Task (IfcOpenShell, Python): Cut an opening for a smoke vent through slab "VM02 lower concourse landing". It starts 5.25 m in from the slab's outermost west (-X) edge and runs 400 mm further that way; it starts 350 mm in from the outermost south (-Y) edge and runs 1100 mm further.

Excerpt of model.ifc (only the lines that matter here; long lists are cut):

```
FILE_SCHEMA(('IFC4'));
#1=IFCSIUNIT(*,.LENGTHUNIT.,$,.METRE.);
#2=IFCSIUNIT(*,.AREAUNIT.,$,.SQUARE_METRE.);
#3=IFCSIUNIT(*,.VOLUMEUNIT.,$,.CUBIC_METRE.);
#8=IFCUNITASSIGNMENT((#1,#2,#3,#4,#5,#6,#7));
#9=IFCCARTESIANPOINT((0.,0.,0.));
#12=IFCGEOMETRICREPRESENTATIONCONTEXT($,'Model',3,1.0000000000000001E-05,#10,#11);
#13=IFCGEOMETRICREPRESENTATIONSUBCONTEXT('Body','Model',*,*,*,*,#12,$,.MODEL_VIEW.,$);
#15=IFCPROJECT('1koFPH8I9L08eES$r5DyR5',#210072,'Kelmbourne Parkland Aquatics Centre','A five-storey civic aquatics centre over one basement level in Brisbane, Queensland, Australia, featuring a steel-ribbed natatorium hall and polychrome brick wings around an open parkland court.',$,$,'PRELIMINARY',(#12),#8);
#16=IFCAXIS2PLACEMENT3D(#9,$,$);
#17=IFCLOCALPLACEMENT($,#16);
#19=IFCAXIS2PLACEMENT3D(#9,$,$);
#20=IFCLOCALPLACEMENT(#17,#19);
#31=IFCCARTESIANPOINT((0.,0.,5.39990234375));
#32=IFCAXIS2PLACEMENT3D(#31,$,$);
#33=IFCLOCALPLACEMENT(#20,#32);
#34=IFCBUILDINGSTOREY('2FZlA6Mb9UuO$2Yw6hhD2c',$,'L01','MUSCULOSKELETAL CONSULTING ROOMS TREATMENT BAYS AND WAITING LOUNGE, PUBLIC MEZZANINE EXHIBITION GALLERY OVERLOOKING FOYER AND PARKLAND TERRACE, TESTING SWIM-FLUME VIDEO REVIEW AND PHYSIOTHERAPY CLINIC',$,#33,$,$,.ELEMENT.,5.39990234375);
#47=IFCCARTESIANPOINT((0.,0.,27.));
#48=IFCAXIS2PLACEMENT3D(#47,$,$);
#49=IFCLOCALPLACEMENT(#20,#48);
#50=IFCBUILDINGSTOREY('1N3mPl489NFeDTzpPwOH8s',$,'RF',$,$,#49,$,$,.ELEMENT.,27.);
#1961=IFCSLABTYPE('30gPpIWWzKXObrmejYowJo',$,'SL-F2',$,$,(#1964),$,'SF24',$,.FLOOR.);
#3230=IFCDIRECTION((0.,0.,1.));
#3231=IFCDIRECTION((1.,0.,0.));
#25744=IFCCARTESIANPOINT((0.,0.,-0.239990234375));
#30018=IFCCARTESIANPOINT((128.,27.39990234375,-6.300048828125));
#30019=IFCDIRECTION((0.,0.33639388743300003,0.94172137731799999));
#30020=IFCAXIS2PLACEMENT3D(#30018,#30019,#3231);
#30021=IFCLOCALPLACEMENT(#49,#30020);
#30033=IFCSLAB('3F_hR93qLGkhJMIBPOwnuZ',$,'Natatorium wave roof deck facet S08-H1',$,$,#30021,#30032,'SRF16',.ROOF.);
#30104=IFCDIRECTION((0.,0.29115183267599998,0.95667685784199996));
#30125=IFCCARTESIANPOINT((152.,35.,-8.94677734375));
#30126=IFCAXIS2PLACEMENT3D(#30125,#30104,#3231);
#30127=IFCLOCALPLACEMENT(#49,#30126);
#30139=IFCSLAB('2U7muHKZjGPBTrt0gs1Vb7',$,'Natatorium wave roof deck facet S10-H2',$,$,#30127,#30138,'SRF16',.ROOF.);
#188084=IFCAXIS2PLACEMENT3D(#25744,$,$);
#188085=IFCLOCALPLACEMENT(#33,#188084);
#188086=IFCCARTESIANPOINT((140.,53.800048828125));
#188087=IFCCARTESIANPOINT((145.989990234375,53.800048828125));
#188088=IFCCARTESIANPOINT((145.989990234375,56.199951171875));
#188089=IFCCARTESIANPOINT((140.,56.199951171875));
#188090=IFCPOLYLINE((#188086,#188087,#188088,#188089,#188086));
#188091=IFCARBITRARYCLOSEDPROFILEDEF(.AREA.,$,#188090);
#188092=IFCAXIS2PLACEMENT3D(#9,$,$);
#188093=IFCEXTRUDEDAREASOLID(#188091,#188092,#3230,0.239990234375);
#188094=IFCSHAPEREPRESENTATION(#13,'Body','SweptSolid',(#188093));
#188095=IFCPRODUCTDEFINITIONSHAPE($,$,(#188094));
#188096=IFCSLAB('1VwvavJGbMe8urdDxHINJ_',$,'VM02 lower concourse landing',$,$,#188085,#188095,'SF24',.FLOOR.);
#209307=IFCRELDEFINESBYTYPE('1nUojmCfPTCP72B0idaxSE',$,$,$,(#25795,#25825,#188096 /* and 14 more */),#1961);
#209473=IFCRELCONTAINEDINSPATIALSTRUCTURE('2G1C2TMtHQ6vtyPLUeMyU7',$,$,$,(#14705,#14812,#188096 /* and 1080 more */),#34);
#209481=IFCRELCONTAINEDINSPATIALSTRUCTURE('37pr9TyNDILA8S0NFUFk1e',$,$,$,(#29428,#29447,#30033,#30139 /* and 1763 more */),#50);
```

```python
import numpy as np
import ifcopenshell
import ifcopenshell.api.feature
import ifcopenshell.api.geometry
import ifcopenshell.api.root
import ifcopenshell.geom
import ifcopenshell.util.placement
import ifcopenshell.util.representation
import ifcopenshell.util.shape
import ifcopenshell.util.unit

model = ifcopenshell.open("model.ifc")
unit_scale = ifcopenshell.util.unit.calculate_unit_scale(model)
settings = ifcopenshell.geom.settings()


def volume(element):
    """Net volume in cubic metres, openings subtracted."""
    shape = ifcopenshell.geom.create_shape(settings, element)
    return ifcopenshell.util.shape.get_volume(shape.geometry)


slab = model.by_guid("1VwvavJGbMe8urdDxHINJ_")
before = volume(slab)

# Extent in the slab's own axes, in metres. The edges named are its -X and -Y sides.
slab_shape = ifcopenshell.geom.create_shape(settings, slab)
vertices = ifcopenshell.util.shape.get_vertices(slab_shape.geometry)
x_min, y_min, bottom = vertices.min(axis=0)
top = vertices[:, 2].max()

opening = ifcopenshell.api.root.create_entity(model, ifc_class="IfcOpeningElement", name="Smoke vent opening", predefined_type="OPENING")
context = ifcopenshell.util.representation.get_context(model, "Model", "Body", "MODEL_VIEW")
width, depth = 0.4, 1.1
outline = [(0.0, 0.0), (width, 0.0), (width, depth), (0.0, depth), (0.0, 0.0)]
# Overshoot both faces by 50 mm so the cut is clean.
shape = ifcopenshell.api.geometry.add_slab_representation(
    model, context=context, depth=top - bottom + 0.1, polyline=outline
)
ifcopenshell.api.geometry.assign_representation(model, product=opening, representation=shape)

matrix = ifcopenshell.util.placement.get_local_placement(slab.ObjectPlacement)
matrix[:, 3] = matrix @ np.append(np.array([x_min + 5.25, y_min + 0.35, bottom - 0.05]) / unit_scale, 1.0)
ifcopenshell.api.geometry.edit_object_placement(model, product=opening, matrix=matrix, is_si=False)
ifcopenshell.api.feature.add_feature(model, feature=opening, element=slab)

after = volume(slab)

print(f"slab volume {before:.3f} -> {after:.3f} m3")

model.write("model-out.ifc")
```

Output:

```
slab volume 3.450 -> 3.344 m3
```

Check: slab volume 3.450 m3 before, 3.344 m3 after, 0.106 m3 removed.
